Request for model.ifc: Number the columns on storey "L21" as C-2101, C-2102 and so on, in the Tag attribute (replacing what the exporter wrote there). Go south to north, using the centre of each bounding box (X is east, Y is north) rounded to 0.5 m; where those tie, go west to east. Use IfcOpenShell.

First a look at what the model holds.

```python
import ifcopenshell
import ifcopenshell.util.element
import ifcopenshell.util.placement

model = ifcopenshell.open("model.ifc")
print(model.schema)
storey = next(s for s in model.by_type("IfcBuildingStorey") if s.Name == "L21")
columns = [e for e in ifcopenshell.util.element.get_decomposition(storey) if e.is_a("IfcColumn")]
for e in sorted(columns, key=lambda e: e.id()):
    origin = ifcopenshell.util.placement.get_local_placement(e.ObjectPlacement)[:3, 3]
    print(e.id(), e.Tag, e.Name, origin.round(2) + 0.0, sep=" | ")
```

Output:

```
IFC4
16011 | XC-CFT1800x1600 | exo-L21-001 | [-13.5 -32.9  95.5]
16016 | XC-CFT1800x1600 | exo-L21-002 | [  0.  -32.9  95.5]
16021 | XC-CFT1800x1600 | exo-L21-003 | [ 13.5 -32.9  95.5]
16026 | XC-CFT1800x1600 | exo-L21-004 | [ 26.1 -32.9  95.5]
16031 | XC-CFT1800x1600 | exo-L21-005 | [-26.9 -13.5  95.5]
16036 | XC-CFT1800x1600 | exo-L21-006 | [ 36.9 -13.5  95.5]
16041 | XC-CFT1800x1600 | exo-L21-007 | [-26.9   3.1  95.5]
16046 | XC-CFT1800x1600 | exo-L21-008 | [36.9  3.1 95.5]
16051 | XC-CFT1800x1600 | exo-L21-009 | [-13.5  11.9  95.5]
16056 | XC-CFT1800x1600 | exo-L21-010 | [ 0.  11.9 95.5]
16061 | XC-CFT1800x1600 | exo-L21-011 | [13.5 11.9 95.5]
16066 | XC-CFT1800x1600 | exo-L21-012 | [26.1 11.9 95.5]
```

```python
import ifcopenshell
import ifcopenshell.geom
import ifcopenshell.util.element
import ifcopenshell.util.shape

model = ifcopenshell.open("model.ifc")
settings = ifcopenshell.geom.settings()
settings.set("use-world-coords", True)


def centre(element):
    shape = ifcopenshell.geom.create_shape(settings, element)
    return ifcopenshell.util.shape.get_bbox_centroid(shape.geometry)


storey = next(s for s in model.by_type("IfcBuildingStorey") if s.Name == "L21")
columns = [e for e in ifcopenshell.util.element.get_decomposition(storey) if e.is_a("IfcColumn")]

# Insertion points can sit at a corner or the storey origin, so sort by the geometry (in metres).
centres = {e: centre(e) for e in columns}
columns.sort(key=lambda e: (round(centres[e][1] / 0.5), centres[e][0]))

for i, e in enumerate(columns, start=1):
    number = f"C-21{i:02d}"
    e.Tag = number
    print(e.id(), number)

model.write("model_v2.ifc")
```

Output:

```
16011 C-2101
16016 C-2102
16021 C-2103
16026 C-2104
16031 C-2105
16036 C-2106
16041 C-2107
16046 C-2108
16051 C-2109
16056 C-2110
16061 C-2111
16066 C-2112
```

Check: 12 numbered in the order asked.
